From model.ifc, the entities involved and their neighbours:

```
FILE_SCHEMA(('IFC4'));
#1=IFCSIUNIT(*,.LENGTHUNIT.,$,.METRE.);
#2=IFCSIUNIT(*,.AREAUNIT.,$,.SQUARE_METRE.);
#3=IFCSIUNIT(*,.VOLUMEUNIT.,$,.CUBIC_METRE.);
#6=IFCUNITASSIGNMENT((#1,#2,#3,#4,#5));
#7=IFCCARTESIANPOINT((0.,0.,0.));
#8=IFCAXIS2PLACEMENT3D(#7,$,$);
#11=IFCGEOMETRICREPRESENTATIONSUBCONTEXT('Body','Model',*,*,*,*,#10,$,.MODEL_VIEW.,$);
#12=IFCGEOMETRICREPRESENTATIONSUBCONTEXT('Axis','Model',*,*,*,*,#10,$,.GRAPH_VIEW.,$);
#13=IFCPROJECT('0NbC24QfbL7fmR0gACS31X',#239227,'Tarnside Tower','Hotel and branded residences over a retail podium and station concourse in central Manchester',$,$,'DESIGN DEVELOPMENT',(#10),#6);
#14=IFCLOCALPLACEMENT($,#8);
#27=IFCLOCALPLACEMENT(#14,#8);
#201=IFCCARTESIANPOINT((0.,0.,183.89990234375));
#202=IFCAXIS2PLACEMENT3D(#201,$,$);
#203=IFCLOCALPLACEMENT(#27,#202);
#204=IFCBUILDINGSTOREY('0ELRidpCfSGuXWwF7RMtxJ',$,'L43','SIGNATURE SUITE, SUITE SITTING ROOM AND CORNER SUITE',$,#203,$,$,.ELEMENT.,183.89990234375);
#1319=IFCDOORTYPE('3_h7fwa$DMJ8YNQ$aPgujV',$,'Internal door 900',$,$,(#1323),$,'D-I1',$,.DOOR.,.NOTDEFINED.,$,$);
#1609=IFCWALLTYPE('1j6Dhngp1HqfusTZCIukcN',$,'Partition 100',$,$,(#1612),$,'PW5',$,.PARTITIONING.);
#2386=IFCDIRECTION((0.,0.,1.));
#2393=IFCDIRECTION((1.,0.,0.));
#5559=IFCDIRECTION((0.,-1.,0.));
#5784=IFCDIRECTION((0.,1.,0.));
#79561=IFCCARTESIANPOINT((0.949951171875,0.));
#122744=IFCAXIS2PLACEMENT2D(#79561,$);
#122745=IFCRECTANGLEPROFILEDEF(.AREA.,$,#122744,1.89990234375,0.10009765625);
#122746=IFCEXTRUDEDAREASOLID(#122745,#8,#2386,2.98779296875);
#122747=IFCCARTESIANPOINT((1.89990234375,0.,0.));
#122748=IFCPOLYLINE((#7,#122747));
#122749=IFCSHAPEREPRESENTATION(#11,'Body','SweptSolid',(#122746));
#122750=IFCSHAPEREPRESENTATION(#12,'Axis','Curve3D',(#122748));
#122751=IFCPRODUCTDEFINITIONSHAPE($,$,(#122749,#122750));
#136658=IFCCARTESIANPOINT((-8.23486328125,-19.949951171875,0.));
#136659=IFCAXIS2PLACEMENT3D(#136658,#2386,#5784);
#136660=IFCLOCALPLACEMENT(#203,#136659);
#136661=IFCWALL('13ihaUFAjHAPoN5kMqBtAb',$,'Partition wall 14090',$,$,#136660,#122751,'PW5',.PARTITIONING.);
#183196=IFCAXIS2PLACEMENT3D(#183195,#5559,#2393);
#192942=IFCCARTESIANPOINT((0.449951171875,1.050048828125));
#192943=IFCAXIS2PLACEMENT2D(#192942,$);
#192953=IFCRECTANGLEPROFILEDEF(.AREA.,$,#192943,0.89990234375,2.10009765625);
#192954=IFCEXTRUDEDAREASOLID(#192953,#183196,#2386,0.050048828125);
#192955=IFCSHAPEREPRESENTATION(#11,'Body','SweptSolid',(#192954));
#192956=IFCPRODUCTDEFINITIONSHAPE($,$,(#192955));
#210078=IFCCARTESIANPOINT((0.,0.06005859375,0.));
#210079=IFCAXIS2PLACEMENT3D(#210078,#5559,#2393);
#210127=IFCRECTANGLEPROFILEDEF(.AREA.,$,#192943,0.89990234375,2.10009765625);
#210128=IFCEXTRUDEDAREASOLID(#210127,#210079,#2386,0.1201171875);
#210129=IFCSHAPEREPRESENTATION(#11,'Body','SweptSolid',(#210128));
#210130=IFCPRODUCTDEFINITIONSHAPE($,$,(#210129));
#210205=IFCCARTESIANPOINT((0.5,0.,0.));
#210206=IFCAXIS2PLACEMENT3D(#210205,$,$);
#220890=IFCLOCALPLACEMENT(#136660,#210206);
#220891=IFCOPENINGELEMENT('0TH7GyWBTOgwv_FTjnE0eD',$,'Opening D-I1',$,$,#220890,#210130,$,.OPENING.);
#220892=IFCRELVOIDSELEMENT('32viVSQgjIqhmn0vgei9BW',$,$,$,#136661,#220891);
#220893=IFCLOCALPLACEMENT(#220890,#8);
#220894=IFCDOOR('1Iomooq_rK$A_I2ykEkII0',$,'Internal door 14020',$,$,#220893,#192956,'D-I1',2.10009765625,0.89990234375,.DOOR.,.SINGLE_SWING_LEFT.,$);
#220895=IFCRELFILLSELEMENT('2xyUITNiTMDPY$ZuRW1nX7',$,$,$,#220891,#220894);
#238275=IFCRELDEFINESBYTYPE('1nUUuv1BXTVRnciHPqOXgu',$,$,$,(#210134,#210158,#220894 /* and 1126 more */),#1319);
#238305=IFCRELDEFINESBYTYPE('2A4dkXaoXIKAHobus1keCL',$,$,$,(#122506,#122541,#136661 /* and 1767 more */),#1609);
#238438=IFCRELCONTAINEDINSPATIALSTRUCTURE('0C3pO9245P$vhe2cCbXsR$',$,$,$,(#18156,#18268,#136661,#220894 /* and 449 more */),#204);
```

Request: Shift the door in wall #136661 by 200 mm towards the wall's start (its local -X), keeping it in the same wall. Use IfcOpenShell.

```python
import ifcopenshell
import ifcopenshell.api.geometry
import ifcopenshell.util.placement

model = ifcopenshell.open("model.ifc")

door = model.by_id(220894)
opening = door.FillsVoids[0].RelatingOpeningElement
wall = opening.VoidsElements[0].RelatingBuildingElement

wall_matrix = ifcopenshell.util.placement.get_local_placement(wall.ObjectPlacement)
shift = wall_matrix[:3, 0] * -0.2
before = ifcopenshell.util.placement.get_local_placement(door.ObjectPlacement)[:3, 3].copy()

# The door is placed relative to its opening, so it follows when the opening moves.
matrix = ifcopenshell.util.placement.get_local_placement(opening.ObjectPlacement)
matrix[:3, 3] += shift
ifcopenshell.api.geometry.edit_object_placement(
    model, product=opening, matrix=matrix, is_si=False, should_transform_children=True
)

after = ifcopenshell.util.placement.get_local_placement(door.ObjectPlacement)[:3, 3]
print("door moved by", (after - before).round(3) + 0.0)

model.write("model_edited.ifc")
```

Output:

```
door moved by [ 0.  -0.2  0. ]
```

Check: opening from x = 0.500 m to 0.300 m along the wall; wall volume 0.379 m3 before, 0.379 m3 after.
